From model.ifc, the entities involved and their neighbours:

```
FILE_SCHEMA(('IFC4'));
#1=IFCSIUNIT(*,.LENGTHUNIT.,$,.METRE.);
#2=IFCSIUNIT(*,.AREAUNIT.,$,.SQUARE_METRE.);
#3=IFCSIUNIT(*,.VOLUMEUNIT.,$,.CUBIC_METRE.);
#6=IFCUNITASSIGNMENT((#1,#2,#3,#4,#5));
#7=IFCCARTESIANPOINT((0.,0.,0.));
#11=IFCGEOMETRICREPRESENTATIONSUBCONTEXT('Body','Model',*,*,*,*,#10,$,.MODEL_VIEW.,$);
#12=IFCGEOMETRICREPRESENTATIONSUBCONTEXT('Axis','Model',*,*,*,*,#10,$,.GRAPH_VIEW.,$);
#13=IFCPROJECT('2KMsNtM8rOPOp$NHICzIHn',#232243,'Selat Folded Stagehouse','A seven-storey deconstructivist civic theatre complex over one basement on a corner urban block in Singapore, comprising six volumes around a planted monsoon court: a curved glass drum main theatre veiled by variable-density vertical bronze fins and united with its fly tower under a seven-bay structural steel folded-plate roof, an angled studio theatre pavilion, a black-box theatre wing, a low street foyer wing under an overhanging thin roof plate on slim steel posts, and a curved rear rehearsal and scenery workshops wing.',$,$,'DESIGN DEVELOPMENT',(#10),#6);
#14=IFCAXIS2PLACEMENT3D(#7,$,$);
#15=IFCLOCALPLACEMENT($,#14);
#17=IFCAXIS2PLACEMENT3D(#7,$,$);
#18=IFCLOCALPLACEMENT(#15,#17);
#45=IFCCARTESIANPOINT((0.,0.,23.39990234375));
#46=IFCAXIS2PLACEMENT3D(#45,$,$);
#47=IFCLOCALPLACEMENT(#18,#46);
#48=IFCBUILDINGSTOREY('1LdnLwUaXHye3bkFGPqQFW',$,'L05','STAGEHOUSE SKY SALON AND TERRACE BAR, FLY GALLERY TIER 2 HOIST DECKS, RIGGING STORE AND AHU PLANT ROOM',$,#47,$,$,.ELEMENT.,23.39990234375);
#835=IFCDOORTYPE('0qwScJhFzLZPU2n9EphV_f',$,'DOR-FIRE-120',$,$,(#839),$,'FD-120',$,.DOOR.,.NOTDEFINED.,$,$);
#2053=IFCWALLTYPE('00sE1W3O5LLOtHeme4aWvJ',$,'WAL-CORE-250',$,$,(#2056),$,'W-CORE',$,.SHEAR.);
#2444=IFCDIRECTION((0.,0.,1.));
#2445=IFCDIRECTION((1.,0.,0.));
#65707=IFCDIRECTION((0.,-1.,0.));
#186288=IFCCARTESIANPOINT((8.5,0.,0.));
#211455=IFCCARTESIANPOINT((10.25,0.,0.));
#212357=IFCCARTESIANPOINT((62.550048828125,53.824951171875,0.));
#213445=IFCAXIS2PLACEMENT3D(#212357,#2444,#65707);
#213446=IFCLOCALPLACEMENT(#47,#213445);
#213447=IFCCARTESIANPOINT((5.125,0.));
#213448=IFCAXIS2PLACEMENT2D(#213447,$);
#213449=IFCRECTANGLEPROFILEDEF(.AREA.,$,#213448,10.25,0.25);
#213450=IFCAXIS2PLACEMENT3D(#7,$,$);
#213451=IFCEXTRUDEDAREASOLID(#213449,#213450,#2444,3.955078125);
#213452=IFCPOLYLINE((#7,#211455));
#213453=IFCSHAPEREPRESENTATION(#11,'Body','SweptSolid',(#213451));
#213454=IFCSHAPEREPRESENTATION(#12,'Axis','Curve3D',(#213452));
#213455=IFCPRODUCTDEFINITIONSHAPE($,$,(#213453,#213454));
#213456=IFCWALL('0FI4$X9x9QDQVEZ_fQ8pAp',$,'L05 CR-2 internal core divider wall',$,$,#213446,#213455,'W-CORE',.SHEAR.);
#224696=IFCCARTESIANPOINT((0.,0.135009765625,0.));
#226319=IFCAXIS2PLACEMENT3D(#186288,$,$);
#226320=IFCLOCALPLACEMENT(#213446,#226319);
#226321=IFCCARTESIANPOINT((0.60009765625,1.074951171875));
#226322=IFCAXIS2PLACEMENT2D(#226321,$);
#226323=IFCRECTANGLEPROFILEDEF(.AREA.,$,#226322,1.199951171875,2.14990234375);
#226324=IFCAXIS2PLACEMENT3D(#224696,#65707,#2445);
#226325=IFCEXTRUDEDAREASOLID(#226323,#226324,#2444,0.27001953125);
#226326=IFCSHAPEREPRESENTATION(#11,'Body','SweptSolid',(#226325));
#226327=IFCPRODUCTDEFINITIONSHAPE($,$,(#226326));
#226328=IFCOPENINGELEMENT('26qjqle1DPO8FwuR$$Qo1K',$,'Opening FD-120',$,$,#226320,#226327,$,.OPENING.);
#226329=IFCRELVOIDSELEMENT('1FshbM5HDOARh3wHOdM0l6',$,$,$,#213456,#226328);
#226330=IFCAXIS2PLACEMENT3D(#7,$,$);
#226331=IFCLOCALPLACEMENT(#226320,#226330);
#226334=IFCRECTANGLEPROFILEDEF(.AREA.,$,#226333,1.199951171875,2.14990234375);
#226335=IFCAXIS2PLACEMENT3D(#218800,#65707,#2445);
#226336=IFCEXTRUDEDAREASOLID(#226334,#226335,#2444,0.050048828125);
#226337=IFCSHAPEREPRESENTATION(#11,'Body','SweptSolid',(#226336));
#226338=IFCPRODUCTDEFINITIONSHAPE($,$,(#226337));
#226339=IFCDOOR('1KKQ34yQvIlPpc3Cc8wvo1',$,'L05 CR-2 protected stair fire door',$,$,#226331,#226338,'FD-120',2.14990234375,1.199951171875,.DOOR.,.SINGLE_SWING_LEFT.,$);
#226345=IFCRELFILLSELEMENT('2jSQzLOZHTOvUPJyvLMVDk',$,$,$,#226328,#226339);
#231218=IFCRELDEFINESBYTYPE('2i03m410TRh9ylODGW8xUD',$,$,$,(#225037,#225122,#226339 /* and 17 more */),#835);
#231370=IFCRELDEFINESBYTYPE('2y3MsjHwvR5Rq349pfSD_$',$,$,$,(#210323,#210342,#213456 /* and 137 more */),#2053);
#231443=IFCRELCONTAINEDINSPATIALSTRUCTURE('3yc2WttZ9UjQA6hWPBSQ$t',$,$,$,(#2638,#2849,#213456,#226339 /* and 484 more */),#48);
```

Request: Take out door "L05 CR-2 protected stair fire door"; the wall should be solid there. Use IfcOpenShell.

```python
import ifcopenshell
import ifcopenshell.api.feature
import ifcopenshell.api.root
import ifcopenshell.geom
import ifcopenshell.util.shape

model = ifcopenshell.open("model.ifc")
settings = ifcopenshell.geom.settings()


def volume(element):
    """Net volume in cubic metres, openings subtracted."""
    shape = ifcopenshell.geom.create_shape(settings, element)
    return ifcopenshell.util.shape.get_volume(shape.geometry)


door = model.by_guid("1KKQ34yQvIlPpc3Cc8wvo1")
opening = door.FillsVoids[0].RelatingOpeningElement
wall = opening.VoidsElements[0].RelatingBuildingElement
before = volume(wall)

ifcopenshell.api.root.remove_product(model, product=door)
ifcopenshell.api.feature.remove_feature(model, feature=opening)

after = volume(wall)

print(f"wall volume {before:.3f} -> {after:.3f} m3")

model.write("model_edited.ifc")
```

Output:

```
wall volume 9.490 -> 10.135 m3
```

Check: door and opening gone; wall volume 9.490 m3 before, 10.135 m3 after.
